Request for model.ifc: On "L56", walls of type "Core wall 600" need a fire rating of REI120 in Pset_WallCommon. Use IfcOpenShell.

First a look at what the model holds.

```python
import ifcopenshell
import ifcopenshell.util.element

model = ifcopenshell.open("model.ifc")
print(model.schema)
storey = next(s for s in model.by_type("IfcBuildingStorey") if s.Name == "L56")
walls = [e for e in ifcopenshell.util.element.get_decomposition(storey) if e.is_a("IfcWall")]
seen = {}
for e in walls:
    element_type = ifcopenshell.util.element.get_type(e)
    key = (element_type.Name if element_type != e and element_type else None, ifcopenshell.util.element.get_pset(e, "Pset_WallCommon", "FireRating"))
    seen[key] = seen.get(key, 0) + 1
for (name, value), count in sorted(seen.items(), key=str):
    print(count, "x", name, "|", value)
```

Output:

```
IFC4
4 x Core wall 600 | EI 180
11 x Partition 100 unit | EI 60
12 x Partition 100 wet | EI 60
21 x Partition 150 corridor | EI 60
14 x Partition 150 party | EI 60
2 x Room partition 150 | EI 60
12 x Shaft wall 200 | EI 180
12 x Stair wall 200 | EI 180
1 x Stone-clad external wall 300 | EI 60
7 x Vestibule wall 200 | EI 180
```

```python
import ifcopenshell
import ifcopenshell.api.pset
import ifcopenshell.util.element

model = ifcopenshell.open("model.ifc")

storey = next(s for s in model.by_type("IfcBuildingStorey") if s.Name == "L56")
walls = [e for e in ifcopenshell.util.element.get_decomposition(storey) if e.is_a("IfcWall")]

count = 0
for e in walls:
    element_type = ifcopenshell.util.element.get_type(e)
    if element_type in (None, e) or element_type.Name != "Core wall 600":
        continue
    found = ifcopenshell.util.element.get_pset(e, "Pset_WallCommon", should_inherit=False)
    if found:
        pset = model.by_id(found["id"])
        if len(ifcopenshell.util.element.get_elements_by_pset(pset)) > 1:
            pset = ifcopenshell.api.pset.unshare_pset(model, products=[e], pset=pset)[0]
    else:
        pset = ifcopenshell.api.pset.add_pset(model, product=e, name="Pset_WallCommon")
    ifcopenshell.api.pset.edit_pset(model, pset=pset, properties={"FireRating": "REI120"})
    count += 1

print(count, "walls updated")

model.write("model_updated.ifc")
```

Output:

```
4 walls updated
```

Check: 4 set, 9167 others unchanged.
